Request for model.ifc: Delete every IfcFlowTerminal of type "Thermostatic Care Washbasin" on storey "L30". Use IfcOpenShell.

First a look at what the model holds.

```python
import ifcopenshell
import ifcopenshell.util.element

model = ifcopenshell.open("model.ifc")
print(model.schema)
storey = next(s for s in model.by_type("IfcBuildingStorey") if s.Name == "L30")
terminals = [e for e in ifcopenshell.util.element.get_decomposition(storey) if e.is_a("IfcFlowTerminal")]
seen = {}
for e in terminals:
    element_type = ifcopenshell.util.element.get_type(e)
    name = element_type.Name if element_type not in (None, e) else None
    seen[name] = seen.get(name, 0) + 1
for name, count in sorted(seen.items(), key=str):
    print(count, "x", name)
```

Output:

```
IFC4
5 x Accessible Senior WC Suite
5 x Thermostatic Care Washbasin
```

```python
import ifcopenshell
import ifcopenshell.api.root
import ifcopenshell.util.element

model = ifcopenshell.open("model.ifc")

storey = next(s for s in model.by_type("IfcBuildingStorey") if s.Name == "L30")
terminals = [e for e in ifcopenshell.util.element.get_decomposition(storey) if e.is_a("IfcFlowTerminal")]
targets = [e for e in terminals if (t := ifcopenshell.util.element.get_type(e)) not in (None, e) and t.Name == "Thermostatic Care Washbasin"]

for e in targets:
    ifcopenshell.api.root.remove_product(model, product=e)
print(len(targets), "removed")

model.write("model_rev.ifc")
```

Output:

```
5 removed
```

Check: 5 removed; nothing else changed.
